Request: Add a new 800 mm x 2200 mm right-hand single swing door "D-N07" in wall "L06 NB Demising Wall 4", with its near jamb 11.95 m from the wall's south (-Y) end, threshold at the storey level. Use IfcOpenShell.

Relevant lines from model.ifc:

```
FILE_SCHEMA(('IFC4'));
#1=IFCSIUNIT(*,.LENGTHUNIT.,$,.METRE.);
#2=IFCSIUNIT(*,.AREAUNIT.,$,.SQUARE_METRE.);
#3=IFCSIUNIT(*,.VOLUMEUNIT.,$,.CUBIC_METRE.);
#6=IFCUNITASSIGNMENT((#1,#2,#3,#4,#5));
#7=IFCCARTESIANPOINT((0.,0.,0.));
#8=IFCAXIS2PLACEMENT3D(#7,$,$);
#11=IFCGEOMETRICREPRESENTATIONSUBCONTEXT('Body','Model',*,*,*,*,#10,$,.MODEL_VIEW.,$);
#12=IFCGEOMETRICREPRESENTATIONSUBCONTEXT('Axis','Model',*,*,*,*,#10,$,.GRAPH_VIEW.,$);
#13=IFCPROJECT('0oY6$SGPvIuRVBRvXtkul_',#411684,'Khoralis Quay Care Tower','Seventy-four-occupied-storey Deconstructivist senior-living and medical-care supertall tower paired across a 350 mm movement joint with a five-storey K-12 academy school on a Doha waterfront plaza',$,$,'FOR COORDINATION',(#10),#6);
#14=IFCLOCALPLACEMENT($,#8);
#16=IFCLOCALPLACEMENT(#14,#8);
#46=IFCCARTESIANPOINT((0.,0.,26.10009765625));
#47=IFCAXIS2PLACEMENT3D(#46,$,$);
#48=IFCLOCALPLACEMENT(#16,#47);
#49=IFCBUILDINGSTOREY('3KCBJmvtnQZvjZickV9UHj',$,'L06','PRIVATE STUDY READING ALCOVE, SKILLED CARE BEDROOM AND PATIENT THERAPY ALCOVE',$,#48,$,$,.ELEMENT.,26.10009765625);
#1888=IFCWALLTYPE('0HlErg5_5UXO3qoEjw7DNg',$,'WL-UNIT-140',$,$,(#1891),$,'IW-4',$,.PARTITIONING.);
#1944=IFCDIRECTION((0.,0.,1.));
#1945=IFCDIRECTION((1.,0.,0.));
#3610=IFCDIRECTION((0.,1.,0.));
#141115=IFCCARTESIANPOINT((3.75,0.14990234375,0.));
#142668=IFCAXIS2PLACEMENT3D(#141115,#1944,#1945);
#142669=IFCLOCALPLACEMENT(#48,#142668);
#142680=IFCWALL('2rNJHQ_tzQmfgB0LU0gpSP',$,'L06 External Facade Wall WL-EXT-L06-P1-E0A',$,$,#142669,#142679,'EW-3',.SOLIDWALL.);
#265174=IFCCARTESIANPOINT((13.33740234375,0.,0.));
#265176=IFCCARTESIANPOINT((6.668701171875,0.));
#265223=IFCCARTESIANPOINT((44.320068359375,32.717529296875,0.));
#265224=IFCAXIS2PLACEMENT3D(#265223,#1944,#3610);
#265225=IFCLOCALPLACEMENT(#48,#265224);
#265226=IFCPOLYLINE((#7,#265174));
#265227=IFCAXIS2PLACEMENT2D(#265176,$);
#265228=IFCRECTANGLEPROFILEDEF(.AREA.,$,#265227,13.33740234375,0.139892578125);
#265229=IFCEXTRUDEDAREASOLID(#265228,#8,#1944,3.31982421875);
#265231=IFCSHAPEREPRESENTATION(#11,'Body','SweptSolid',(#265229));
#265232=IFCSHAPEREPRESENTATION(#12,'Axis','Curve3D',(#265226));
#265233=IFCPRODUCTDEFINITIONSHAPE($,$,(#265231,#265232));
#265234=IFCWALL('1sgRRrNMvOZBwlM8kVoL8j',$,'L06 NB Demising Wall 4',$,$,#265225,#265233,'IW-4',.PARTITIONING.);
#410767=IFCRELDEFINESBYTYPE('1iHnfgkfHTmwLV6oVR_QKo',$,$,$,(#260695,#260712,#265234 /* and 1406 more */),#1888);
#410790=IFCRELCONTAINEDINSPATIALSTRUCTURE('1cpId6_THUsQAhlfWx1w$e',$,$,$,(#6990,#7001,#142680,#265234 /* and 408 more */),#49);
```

```python
import numpy as np
import ifcopenshell
import ifcopenshell.api.feature
import ifcopenshell.api.geometry
import ifcopenshell.api.root
import ifcopenshell.api.spatial
import ifcopenshell.geom
import ifcopenshell.util.element
import ifcopenshell.util.placement
import ifcopenshell.util.representation
import ifcopenshell.util.shape
import ifcopenshell.util.unit

model = ifcopenshell.open("model.ifc")
unit_scale = ifcopenshell.util.unit.calculate_unit_scale(model)
settings = ifcopenshell.geom.settings()


def volume(element):
    """Net volume in cubic metres, openings subtracted."""
    shape = ifcopenshell.geom.create_shape(settings, element)
    return ifcopenshell.util.shape.get_volume(shape.geometry)


wall = model.by_guid("1sgRRrNMvOZBwlM8kVoL8j")
storey = ifcopenshell.util.element.get_container(wall, ifc_class="IfcBuildingStorey")
context = ifcopenshell.util.representation.get_context(model, "Model", "Body", "MODEL_VIEW")
before = volume(wall)

width, height, from_end, sill = 0.8, 2.2, 11.95, 0.0  # metres

# The wall runs along its own X axis, and the end named is its -X end.
wall_shape = ifcopenshell.geom.create_shape(settings, wall)
x, y, z = ifcopenshell.util.shape.get_vertices(wall_shape.geometry).T
start = x.min() + from_end
face, thickness = float(y.min()), float(y.max() - y.min())
wall_matrix = ifcopenshell.util.placement.get_local_placement(wall.ObjectPlacement)
level = ifcopenshell.util.placement.get_local_placement(storey.ObjectPlacement)[2, 3]


def in_wall(x, y):
    """Placement at x, y metres in the wall's axes, at sill height."""
    matrix = wall_matrix.copy()
    matrix[:, 3] = wall_matrix @ np.array([x / unit_scale, y / unit_scale, 0.0, 1.0])
    matrix[2, 3] = level + sill / unit_scale
    return matrix


# Opening: a box that overshoots both wall faces by 50 mm.
opening = ifcopenshell.api.root.create_entity(model, ifc_class="IfcOpeningElement", predefined_type="OPENING")
box = ifcopenshell.api.geometry.add_wall_representation(
    model, context=context, length=width, height=height, thickness=thickness + 0.1
)
ifcopenshell.api.geometry.assign_representation(model, product=opening, representation=box)
ifcopenshell.api.geometry.edit_object_placement(model, product=opening, matrix=in_wall(start, face - 0.05), is_si=False)
ifcopenshell.api.feature.add_feature(model, feature=opening, element=wall)

door = ifcopenshell.api.root.create_entity(model, ifc_class="IfcDoor", name="D-N07", predefined_type="DOOR")
door.OverallWidth, door.OverallHeight = width / unit_scale, height / unit_scale
door.OperationType = "SINGLE_SWING_RIGHT"
body = ifcopenshell.api.geometry.add_door_representation(
    model,
    context=context,
    overall_width=door.OverallWidth,
    overall_height=door.OverallHeight,
    operation_type="SINGLE_SWING_RIGHT",
    lining_properties={"LiningDepth": thickness / unit_scale, "ThresholdDepth": thickness / unit_scale},
)
ifcopenshell.api.geometry.assign_representation(model, product=door, representation=body)
ifcopenshell.api.spatial.assign_container(model, products=[door], relating_structure=storey)
ifcopenshell.api.feature.add_filling(model, opening=opening, element=door)

# The lining spans the wall, so the door starts at the wall face.
ifcopenshell.api.geometry.edit_object_placement(model, product=door, matrix=in_wall(start, face), is_si=False)

after = volume(wall)

print(f"wall volume {before:.3f} -> {after:.3f} m3")

model.write("model_edited.ifc")
```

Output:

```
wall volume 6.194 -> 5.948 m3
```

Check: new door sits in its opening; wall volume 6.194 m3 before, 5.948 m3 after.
